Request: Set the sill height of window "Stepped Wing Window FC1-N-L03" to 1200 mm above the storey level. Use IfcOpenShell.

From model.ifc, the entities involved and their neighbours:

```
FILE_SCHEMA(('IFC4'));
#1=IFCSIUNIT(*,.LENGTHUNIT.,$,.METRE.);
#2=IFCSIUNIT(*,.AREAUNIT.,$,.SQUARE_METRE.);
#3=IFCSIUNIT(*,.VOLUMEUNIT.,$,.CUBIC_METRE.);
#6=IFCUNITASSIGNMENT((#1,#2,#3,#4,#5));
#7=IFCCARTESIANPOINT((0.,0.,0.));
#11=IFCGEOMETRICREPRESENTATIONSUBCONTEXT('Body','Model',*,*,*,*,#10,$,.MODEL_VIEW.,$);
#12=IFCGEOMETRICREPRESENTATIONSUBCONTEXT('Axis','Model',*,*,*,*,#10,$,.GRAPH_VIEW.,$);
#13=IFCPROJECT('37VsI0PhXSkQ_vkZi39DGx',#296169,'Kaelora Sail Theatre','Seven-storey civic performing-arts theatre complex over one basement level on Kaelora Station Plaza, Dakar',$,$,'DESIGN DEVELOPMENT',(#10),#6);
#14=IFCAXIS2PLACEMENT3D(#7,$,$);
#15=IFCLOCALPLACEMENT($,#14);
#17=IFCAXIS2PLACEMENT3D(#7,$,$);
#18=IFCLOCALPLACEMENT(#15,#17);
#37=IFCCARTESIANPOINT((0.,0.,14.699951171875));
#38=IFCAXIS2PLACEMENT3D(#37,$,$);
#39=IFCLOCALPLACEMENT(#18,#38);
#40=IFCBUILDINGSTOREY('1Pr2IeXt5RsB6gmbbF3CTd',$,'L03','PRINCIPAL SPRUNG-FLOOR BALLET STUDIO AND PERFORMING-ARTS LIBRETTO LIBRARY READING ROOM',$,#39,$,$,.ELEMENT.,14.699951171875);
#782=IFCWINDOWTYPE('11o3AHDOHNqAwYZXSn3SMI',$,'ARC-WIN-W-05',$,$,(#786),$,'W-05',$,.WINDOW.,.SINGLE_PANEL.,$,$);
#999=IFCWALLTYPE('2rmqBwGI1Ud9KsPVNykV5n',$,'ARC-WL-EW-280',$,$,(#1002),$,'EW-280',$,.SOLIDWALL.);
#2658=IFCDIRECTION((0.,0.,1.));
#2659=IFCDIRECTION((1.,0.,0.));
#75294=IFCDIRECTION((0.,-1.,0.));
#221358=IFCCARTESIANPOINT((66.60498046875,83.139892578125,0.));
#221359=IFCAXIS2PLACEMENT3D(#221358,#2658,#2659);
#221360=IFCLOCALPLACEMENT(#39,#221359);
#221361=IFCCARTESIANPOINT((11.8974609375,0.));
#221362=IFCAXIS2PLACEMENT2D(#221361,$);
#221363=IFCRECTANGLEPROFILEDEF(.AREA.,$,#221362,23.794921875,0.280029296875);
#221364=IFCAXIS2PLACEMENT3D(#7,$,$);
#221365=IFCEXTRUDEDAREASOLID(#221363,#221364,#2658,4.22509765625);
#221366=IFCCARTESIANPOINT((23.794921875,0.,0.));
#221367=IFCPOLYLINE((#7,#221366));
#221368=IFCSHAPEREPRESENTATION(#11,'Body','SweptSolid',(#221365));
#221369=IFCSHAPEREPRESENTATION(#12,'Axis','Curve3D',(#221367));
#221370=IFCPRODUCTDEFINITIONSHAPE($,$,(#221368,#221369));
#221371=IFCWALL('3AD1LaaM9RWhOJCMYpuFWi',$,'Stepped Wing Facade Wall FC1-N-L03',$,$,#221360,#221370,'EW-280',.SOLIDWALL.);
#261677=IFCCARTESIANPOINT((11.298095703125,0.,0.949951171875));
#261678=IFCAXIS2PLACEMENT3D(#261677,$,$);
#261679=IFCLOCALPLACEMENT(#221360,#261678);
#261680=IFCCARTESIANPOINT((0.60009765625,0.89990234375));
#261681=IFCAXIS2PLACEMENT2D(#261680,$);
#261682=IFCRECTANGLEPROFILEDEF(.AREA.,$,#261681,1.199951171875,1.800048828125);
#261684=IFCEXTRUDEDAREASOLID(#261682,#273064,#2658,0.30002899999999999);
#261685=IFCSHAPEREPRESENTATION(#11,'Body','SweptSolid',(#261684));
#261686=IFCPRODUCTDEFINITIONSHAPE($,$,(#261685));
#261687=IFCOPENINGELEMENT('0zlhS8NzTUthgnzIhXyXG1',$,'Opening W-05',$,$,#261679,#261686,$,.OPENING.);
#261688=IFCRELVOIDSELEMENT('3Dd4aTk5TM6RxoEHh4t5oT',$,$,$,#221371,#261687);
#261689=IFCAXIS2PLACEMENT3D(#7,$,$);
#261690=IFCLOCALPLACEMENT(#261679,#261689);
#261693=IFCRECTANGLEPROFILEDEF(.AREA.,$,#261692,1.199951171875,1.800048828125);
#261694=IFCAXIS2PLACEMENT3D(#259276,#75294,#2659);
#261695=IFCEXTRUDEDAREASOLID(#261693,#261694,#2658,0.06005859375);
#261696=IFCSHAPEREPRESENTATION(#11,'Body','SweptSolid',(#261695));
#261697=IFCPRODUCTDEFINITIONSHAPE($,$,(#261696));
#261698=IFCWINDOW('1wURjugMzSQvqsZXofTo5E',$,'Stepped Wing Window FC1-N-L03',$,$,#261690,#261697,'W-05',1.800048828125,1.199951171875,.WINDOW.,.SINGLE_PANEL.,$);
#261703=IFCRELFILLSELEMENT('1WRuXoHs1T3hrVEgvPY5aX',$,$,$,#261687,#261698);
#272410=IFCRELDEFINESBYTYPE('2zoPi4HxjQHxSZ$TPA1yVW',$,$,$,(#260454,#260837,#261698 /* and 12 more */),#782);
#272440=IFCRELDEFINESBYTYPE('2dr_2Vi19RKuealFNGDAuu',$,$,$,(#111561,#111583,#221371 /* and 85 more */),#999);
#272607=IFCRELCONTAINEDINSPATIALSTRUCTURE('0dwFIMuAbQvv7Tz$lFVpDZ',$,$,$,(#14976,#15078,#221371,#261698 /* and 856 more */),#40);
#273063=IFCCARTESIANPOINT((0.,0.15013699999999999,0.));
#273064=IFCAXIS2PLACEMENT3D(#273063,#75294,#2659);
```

```python
import numpy as np
import ifcopenshell
import ifcopenshell.api.geometry
import ifcopenshell.geom
import ifcopenshell.util.element
import ifcopenshell.util.placement
import ifcopenshell.util.shape
import ifcopenshell.util.unit

model = ifcopenshell.open("model.ifc")
unit_scale = ifcopenshell.util.unit.calculate_unit_scale(model)

window = model.by_guid("1wURjugMzSQvqsZXofTo5E")
opening = window.FillsVoids[0].RelatingOpeningElement
storey = ifcopenshell.util.element.get_container(window, ifc_class="IfcBuildingStorey")
level = ifcopenshell.util.placement.get_local_placement(storey.ObjectPlacement)[2, 3]

# The opening's origin need not be at the sill, so measure its lowest point.
shape = ifcopenshell.geom.create_shape(ifcopenshell.geom.settings(), opening)
bottom = ifcopenshell.util.shape.get_shape_bottom_elevation(shape, shape.geometry) / unit_scale
dz = level + 1.2 / unit_scale - bottom

shift = np.array([0.0, 0.0, dz])
# The window is placed relative to its opening, so it follows when the opening moves.
matrix = ifcopenshell.util.placement.get_local_placement(opening.ObjectPlacement)
matrix[:3, 3] += shift
ifcopenshell.api.geometry.edit_object_placement(
    model, product=opening, matrix=matrix, is_si=False, should_transform_children=True
)

print(f"moved by {dz * unit_scale:+.3f} m")

model.write("model-out.ifc")
```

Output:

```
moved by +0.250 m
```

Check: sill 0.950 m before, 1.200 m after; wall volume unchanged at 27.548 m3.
